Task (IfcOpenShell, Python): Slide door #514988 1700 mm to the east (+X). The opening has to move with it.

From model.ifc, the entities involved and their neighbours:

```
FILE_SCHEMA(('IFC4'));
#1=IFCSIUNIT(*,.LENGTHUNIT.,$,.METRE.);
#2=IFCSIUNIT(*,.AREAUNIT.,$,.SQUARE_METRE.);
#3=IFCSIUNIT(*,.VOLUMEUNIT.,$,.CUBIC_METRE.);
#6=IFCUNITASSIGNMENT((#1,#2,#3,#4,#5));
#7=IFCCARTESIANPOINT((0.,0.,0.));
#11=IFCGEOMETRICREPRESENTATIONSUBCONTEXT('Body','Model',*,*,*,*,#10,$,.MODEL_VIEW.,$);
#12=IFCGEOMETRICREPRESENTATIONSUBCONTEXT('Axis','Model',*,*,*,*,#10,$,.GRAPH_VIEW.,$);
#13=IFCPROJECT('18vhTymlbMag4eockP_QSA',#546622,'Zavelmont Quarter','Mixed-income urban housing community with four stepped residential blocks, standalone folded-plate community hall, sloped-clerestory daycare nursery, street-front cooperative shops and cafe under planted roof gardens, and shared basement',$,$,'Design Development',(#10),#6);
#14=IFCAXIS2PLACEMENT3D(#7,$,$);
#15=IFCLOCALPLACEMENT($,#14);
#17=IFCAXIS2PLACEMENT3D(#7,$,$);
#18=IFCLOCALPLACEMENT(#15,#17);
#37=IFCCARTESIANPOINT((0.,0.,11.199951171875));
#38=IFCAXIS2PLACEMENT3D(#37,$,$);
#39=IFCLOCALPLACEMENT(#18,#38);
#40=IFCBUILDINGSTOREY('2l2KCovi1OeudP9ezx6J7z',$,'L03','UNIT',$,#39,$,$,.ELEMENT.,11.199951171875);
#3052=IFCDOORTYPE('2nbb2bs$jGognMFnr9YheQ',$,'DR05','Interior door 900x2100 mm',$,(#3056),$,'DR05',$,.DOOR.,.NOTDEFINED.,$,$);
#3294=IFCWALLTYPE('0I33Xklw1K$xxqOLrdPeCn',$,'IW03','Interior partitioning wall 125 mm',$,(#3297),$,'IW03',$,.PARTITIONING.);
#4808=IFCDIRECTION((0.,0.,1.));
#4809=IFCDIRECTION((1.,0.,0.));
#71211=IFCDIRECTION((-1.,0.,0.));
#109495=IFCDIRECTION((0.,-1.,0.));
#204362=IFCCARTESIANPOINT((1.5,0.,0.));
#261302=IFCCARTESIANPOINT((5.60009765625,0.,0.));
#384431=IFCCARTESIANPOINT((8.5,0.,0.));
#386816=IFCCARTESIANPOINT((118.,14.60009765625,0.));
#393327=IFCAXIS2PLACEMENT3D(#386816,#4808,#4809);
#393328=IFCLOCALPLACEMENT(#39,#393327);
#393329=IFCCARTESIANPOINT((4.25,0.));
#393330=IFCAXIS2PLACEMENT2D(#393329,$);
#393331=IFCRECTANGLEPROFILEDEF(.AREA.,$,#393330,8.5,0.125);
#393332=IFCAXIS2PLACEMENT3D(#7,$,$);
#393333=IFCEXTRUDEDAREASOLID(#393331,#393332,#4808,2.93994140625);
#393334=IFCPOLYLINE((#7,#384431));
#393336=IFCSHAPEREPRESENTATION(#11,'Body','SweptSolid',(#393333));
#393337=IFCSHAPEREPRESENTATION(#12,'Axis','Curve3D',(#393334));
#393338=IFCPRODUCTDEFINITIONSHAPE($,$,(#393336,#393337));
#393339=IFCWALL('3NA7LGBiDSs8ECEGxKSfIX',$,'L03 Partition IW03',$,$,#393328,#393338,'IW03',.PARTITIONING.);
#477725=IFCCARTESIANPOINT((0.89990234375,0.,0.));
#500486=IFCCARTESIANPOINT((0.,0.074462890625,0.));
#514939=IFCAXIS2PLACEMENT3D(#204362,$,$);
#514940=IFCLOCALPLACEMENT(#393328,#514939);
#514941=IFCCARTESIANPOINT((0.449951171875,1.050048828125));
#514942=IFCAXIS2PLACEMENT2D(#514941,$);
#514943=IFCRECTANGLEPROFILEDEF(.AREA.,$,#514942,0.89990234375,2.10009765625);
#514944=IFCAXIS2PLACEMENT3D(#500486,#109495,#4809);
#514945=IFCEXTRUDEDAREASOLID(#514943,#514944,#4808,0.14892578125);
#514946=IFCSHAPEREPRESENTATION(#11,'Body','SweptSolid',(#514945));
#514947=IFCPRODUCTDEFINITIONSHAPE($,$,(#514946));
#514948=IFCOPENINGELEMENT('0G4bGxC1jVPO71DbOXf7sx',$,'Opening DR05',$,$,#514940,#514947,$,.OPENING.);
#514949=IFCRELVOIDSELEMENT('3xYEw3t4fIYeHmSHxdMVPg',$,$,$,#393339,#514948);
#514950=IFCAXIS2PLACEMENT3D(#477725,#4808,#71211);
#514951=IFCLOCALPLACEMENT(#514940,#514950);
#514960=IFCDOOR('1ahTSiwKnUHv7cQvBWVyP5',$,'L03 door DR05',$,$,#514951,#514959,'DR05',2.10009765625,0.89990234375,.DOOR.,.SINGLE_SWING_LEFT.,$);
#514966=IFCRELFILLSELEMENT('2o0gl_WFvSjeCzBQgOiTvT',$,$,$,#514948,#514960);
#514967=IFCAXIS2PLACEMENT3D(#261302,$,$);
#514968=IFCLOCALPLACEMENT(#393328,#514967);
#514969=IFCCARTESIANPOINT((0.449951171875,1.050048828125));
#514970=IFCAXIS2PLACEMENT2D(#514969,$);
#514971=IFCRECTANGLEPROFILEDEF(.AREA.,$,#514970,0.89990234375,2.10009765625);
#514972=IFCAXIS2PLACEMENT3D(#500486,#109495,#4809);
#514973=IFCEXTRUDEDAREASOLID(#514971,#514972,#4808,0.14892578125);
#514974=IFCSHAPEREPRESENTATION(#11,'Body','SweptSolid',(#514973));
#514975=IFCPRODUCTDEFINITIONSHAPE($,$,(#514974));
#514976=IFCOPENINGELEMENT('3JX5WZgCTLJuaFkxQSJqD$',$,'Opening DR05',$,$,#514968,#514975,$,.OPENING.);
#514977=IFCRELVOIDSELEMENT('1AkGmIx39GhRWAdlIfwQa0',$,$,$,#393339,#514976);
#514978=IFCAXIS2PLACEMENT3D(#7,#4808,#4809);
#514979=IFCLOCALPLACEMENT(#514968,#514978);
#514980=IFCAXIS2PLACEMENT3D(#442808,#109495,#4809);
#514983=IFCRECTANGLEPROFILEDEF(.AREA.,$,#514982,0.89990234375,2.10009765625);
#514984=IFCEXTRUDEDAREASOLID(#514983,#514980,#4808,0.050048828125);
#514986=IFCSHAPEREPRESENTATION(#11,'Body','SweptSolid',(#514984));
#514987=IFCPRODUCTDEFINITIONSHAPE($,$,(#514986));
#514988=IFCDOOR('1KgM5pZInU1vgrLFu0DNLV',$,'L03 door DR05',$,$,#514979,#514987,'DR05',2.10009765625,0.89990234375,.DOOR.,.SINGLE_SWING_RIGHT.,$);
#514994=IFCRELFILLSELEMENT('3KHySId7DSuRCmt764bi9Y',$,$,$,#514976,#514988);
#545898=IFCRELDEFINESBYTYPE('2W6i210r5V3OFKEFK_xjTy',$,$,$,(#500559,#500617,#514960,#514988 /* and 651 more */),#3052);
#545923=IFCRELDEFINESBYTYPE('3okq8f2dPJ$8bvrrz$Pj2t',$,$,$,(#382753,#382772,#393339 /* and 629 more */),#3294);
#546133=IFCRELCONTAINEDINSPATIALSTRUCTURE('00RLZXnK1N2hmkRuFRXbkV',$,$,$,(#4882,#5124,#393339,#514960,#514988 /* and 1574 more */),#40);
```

```python
import ifcopenshell
import ifcopenshell.api.geometry
import ifcopenshell.util.placement
import ifcopenshell.util.unit

model = ifcopenshell.open("model.ifc")
unit_scale = ifcopenshell.util.unit.calculate_unit_scale(model)

door = model.by_guid("1KgM5pZInU1vgrLFu0DNLV")
opening = door.FillsVoids[0].RelatingOpeningElement
wall = opening.VoidsElements[0].RelatingBuildingElement

wall_matrix = ifcopenshell.util.placement.get_local_placement(wall.ObjectPlacement)
shift = wall_matrix[:3, 0] * 1.7 / unit_scale
before = ifcopenshell.util.placement.get_local_placement(door.ObjectPlacement)[:3, 3].copy()

# The door is placed relative to its opening, so it follows when the opening moves.
matrix = ifcopenshell.util.placement.get_local_placement(opening.ObjectPlacement)
matrix[:3, 3] += shift
ifcopenshell.api.geometry.edit_object_placement(
    model, product=opening, matrix=matrix, is_si=False, should_transform_children=True
)

after = ifcopenshell.util.placement.get_local_placement(door.ObjectPlacement)[:3, 3]
print("door moved by", (after - before).round(3) + 0.0)

model.write("model_edited.ifc")
```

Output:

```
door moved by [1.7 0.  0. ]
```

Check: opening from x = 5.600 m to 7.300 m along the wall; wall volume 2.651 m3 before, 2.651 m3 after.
